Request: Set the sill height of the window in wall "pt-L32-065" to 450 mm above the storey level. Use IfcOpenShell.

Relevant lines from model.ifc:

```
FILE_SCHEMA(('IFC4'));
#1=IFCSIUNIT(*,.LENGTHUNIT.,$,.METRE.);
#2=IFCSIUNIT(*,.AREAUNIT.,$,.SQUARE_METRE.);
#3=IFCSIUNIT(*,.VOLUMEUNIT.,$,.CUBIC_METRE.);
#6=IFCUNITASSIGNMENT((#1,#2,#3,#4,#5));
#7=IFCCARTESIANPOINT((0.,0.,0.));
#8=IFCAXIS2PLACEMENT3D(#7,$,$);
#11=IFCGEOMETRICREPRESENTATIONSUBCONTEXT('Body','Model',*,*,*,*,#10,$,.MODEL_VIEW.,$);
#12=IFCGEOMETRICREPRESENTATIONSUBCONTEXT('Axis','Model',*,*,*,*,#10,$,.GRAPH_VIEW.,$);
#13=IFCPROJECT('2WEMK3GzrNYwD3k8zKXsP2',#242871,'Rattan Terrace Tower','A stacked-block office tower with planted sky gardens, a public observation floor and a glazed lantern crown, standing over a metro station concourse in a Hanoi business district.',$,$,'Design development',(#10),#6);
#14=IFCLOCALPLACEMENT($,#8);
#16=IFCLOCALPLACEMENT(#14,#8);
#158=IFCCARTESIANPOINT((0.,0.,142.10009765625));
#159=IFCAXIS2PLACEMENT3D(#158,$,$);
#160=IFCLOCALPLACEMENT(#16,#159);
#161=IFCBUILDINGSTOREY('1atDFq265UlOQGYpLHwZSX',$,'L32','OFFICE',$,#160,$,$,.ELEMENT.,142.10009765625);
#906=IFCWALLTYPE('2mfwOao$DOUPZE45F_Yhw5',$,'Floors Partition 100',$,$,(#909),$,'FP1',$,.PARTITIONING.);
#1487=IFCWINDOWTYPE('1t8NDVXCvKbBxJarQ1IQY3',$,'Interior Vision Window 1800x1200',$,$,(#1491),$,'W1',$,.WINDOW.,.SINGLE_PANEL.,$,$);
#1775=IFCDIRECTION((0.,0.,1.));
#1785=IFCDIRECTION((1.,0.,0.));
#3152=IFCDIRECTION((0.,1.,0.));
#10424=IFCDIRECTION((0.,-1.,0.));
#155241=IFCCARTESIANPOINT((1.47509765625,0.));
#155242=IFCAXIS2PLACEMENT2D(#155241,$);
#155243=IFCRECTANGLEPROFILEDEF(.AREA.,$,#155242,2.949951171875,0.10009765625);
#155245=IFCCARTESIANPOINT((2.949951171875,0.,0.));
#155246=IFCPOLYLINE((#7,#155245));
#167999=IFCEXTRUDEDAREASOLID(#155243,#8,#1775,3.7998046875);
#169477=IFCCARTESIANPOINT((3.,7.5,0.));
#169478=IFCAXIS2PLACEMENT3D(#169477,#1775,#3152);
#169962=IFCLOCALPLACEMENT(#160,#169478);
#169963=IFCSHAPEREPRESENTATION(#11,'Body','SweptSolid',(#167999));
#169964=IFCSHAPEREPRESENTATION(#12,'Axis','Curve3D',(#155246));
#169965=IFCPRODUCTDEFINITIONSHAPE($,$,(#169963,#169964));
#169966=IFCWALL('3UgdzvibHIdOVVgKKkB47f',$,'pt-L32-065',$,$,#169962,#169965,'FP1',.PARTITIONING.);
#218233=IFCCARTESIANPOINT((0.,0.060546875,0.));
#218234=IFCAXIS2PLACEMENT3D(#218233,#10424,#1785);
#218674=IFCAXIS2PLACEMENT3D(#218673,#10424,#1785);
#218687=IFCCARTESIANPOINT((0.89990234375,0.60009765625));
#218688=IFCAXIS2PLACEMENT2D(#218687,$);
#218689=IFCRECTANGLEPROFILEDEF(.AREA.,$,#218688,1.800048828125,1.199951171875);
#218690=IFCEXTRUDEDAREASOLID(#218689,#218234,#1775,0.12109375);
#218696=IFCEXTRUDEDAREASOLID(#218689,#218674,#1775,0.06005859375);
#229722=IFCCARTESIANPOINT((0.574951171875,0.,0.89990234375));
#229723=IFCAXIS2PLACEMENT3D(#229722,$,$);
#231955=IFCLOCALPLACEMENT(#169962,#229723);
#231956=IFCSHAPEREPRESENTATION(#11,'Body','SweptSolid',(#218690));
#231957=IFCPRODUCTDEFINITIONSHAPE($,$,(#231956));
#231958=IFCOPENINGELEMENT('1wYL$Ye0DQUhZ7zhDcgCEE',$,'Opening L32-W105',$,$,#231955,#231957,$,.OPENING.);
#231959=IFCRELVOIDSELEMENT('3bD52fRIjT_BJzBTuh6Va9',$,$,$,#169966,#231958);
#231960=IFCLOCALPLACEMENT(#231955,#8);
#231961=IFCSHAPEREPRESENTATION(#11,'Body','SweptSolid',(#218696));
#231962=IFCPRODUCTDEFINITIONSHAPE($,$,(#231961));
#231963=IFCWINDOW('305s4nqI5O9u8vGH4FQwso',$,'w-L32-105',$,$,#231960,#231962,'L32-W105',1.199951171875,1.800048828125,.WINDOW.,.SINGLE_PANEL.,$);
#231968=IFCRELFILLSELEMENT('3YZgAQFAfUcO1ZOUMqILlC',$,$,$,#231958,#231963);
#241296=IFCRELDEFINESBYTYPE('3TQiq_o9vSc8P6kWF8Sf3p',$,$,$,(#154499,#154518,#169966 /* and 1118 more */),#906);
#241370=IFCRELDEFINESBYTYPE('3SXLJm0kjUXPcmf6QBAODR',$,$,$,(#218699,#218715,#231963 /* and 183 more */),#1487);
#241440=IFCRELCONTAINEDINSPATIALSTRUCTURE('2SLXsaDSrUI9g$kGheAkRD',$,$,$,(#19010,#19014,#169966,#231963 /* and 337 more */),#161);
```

```python
import numpy as np
import ifcopenshell
import ifcopenshell.api.geometry
import ifcopenshell.geom
import ifcopenshell.util.element
import ifcopenshell.util.placement
import ifcopenshell.util.shape
import ifcopenshell.util.unit

model = ifcopenshell.open("model.ifc")
unit_scale = ifcopenshell.util.unit.calculate_unit_scale(model)

window = model.by_guid("305s4nqI5O9u8vGH4FQwso")
opening = window.FillsVoids[0].RelatingOpeningElement
storey = ifcopenshell.util.element.get_container(window, ifc_class="IfcBuildingStorey")
level = ifcopenshell.util.placement.get_local_placement(storey.ObjectPlacement)[2, 3]

# The opening's origin need not be at the sill, so measure its lowest point.
shape = ifcopenshell.geom.create_shape(ifcopenshell.geom.settings(), opening)
bottom = ifcopenshell.util.shape.get_shape_bottom_elevation(shape, shape.geometry) / unit_scale
dz = level + 0.45 / unit_scale - bottom

shift = np.array([0.0, 0.0, dz])
# The window is placed relative to its opening, so it follows when the opening moves.
matrix = ifcopenshell.util.placement.get_local_placement(opening.ObjectPlacement)
matrix[:3, 3] += shift
ifcopenshell.api.geometry.edit_object_placement(
    model, product=opening, matrix=matrix, is_si=False, should_transform_children=True
)

print(f"moved by {dz * unit_scale:+.3f} m")

model.write("model_v2.ifc")
```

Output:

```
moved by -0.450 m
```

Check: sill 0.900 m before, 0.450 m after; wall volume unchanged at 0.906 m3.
